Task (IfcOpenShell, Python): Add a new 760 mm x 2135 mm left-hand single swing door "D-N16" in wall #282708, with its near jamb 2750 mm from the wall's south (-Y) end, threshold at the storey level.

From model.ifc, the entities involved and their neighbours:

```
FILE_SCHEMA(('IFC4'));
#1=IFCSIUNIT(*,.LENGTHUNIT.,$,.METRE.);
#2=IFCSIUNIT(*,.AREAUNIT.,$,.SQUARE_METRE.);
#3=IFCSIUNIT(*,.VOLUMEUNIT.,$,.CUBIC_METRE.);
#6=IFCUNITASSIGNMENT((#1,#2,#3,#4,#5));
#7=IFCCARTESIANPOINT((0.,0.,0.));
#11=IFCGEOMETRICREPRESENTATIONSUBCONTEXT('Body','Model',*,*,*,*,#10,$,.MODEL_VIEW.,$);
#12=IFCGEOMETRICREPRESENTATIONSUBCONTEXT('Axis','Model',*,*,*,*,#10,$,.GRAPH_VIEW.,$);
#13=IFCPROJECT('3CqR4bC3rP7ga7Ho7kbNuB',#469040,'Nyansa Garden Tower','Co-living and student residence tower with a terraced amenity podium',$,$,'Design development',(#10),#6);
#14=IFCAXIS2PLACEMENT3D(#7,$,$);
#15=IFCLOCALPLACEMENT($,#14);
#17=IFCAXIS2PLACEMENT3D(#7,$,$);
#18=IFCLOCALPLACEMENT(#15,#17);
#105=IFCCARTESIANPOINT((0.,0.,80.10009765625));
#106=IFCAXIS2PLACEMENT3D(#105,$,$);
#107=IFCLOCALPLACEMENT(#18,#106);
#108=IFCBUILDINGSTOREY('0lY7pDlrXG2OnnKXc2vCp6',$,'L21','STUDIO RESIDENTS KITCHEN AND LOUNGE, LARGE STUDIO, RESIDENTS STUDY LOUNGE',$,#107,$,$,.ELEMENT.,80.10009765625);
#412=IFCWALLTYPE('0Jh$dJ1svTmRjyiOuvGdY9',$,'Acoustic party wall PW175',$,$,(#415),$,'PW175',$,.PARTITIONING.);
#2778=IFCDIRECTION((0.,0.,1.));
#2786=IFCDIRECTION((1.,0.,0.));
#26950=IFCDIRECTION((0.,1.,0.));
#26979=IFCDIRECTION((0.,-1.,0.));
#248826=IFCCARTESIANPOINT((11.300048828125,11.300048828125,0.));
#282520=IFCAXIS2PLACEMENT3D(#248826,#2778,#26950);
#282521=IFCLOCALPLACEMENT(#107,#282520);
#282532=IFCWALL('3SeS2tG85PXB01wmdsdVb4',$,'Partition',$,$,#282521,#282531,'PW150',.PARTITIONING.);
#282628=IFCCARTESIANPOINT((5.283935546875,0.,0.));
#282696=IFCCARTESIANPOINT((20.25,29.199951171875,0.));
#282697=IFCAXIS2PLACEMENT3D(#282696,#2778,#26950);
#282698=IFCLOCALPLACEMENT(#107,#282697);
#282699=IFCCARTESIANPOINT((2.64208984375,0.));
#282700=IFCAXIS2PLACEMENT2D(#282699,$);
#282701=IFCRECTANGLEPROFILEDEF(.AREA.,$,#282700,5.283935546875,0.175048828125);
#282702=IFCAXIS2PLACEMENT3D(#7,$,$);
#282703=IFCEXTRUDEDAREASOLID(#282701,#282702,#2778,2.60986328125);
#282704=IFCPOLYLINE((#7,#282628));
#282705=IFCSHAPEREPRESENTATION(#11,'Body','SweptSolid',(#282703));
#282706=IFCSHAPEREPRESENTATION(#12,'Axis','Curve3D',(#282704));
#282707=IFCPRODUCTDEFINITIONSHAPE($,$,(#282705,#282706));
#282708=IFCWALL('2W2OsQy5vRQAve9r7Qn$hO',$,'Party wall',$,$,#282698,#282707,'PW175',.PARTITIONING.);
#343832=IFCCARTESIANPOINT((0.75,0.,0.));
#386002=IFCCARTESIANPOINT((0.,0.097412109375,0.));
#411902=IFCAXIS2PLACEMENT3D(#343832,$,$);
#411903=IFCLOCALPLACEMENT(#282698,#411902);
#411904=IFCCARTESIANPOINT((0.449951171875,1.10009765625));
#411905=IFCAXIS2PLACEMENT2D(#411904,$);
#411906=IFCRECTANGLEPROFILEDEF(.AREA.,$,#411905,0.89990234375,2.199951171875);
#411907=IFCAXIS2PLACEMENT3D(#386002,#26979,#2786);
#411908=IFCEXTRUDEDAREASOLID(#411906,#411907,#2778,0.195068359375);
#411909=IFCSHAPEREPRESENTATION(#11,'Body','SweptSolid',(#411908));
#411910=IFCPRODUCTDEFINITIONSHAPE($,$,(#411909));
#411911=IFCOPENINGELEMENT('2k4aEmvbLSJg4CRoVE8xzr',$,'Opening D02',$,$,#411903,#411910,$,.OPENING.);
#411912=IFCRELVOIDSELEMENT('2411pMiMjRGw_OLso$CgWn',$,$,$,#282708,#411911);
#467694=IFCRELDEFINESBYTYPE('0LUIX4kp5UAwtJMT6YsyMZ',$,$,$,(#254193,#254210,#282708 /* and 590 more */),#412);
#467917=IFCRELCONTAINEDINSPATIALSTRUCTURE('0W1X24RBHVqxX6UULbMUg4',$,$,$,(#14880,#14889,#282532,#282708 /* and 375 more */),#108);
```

```python
import numpy as np
import ifcopenshell
import ifcopenshell.api.feature
import ifcopenshell.api.geometry
import ifcopenshell.api.root
import ifcopenshell.api.spatial
import ifcopenshell.geom
import ifcopenshell.util.element
import ifcopenshell.util.placement
import ifcopenshell.util.representation
import ifcopenshell.util.shape
import ifcopenshell.util.unit

model = ifcopenshell.open("model.ifc")
unit_scale = ifcopenshell.util.unit.calculate_unit_scale(model)
settings = ifcopenshell.geom.settings()


def volume(element):
    """Net volume in cubic metres, openings subtracted."""
    shape = ifcopenshell.geom.create_shape(settings, element)
    return ifcopenshell.util.shape.get_volume(shape.geometry)


wall = model.by_guid("2W2OsQy5vRQAve9r7Qn$hO")
storey = ifcopenshell.util.element.get_container(wall, ifc_class="IfcBuildingStorey")
context = ifcopenshell.util.representation.get_context(model, "Model", "Body", "MODEL_VIEW")
before = volume(wall)

width, height, from_end, sill = 0.76, 2.135, 2.75, 0.0  # metres

# The wall runs along its own X axis, and the end named is its -X end.
wall_shape = ifcopenshell.geom.create_shape(settings, wall)
x, y, z = ifcopenshell.util.shape.get_vertices(wall_shape.geometry).T
start = x.min() + from_end
face, thickness = float(y.min()), float(y.max() - y.min())
wall_matrix = ifcopenshell.util.placement.get_local_placement(wall.ObjectPlacement)
level = ifcopenshell.util.placement.get_local_placement(storey.ObjectPlacement)[2, 3]


def in_wall(x, y):
    """Placement at x, y metres in the wall's axes, at sill height."""
    matrix = wall_matrix.copy()
    matrix[:, 3] = wall_matrix @ np.array([x / unit_scale, y / unit_scale, 0.0, 1.0])
    matrix[2, 3] = level + sill / unit_scale
    return matrix


# Opening: a box that overshoots both wall faces by 50 mm.
opening = ifcopenshell.api.root.create_entity(model, ifc_class="IfcOpeningElement", predefined_type="OPENING")
box = ifcopenshell.api.geometry.add_wall_representation(
    model, context=context, length=width, height=height, thickness=thickness + 0.1
)
ifcopenshell.api.geometry.assign_representation(model, product=opening, representation=box)
ifcopenshell.api.geometry.edit_object_placement(model, product=opening, matrix=in_wall(start, face - 0.05), is_si=False)
ifcopenshell.api.feature.add_feature(model, feature=opening, element=wall)

door = ifcopenshell.api.root.create_entity(model, ifc_class="IfcDoor", name="D-N16", predefined_type="DOOR")
door.OverallWidth, door.OverallHeight = width / unit_scale, height / unit_scale
door.OperationType = "SINGLE_SWING_LEFT"
body = ifcopenshell.api.geometry.add_door_representation(
    model,
    context=context,
    overall_width=door.OverallWidth,
    overall_height=door.OverallHeight,
    operation_type="SINGLE_SWING_LEFT",
    lining_properties={"LiningDepth": thickness / unit_scale, "ThresholdDepth": thickness / unit_scale},
)
ifcopenshell.api.geometry.assign_representation(model, product=door, representation=body)
ifcopenshell.api.spatial.assign_container(model, products=[door], relating_structure=storey)
ifcopenshell.api.feature.add_filling(model, opening=opening, element=door)

# The lining spans the wall, so the door starts at the wall face.
ifcopenshell.api.geometry.edit_object_placement(model, product=door, matrix=in_wall(start, face), is_si=False)

after = volume(wall)

print(f"wall volume {before:.3f} -> {after:.3f} m3")

model.write("model_updated.ifc")
```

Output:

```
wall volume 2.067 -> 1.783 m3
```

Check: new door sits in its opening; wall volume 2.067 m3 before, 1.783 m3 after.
